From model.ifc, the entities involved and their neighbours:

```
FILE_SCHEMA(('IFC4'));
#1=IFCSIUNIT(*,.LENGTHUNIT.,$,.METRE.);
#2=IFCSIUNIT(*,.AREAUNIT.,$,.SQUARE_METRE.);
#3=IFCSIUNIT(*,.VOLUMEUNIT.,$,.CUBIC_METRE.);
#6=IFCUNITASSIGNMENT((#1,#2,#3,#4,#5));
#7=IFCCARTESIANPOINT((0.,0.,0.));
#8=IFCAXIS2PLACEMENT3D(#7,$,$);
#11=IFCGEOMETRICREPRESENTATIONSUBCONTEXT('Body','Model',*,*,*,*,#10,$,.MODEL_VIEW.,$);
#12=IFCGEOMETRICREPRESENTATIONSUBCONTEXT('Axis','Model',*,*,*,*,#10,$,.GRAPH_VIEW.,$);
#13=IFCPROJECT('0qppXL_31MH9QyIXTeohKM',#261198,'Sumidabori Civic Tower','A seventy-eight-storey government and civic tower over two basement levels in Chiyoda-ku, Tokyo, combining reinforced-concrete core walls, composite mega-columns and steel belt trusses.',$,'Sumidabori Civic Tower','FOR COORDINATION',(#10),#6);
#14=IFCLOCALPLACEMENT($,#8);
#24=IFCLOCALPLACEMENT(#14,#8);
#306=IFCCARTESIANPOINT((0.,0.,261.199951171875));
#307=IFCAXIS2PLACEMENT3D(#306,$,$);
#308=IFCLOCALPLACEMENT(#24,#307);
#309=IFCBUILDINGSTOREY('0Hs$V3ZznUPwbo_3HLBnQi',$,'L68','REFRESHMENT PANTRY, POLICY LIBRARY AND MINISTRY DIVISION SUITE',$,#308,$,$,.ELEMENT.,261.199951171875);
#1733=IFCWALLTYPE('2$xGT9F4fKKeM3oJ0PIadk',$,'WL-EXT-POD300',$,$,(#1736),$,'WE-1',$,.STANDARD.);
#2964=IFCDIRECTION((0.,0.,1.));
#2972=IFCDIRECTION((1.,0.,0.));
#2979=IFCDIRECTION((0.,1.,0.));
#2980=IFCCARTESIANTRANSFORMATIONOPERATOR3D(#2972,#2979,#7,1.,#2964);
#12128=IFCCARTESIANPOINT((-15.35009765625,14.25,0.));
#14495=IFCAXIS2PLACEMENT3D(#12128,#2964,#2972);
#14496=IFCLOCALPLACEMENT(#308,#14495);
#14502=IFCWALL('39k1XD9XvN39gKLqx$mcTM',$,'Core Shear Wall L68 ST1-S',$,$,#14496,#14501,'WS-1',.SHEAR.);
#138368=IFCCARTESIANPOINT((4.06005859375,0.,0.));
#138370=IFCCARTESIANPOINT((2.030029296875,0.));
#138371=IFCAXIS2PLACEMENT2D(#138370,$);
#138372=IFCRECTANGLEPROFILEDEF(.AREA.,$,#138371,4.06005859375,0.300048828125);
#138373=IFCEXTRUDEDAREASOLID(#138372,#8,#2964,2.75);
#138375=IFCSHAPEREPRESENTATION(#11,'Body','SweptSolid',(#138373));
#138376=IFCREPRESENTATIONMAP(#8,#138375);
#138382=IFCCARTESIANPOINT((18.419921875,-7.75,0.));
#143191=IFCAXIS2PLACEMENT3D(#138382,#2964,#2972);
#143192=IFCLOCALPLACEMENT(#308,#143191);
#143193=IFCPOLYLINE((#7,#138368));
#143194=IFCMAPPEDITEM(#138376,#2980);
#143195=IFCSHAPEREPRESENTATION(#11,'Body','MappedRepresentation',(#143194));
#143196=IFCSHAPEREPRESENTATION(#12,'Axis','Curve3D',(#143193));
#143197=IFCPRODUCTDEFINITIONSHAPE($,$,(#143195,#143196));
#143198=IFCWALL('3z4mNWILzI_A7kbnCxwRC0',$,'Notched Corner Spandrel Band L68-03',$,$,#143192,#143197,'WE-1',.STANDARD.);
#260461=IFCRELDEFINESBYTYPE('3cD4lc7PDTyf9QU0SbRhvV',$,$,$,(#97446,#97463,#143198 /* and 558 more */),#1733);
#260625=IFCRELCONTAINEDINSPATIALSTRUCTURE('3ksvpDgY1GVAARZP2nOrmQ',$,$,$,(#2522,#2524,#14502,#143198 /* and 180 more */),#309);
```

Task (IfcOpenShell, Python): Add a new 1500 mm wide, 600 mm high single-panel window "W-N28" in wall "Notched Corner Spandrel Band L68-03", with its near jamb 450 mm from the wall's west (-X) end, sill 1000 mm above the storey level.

```python
import numpy as np
import ifcopenshell
import ifcopenshell.api.feature
import ifcopenshell.api.geometry
import ifcopenshell.api.root
import ifcopenshell.api.spatial
import ifcopenshell.geom
import ifcopenshell.util.element
import ifcopenshell.util.placement
import ifcopenshell.util.representation
import ifcopenshell.util.shape
import ifcopenshell.util.unit

model = ifcopenshell.open("model.ifc")
unit_scale = ifcopenshell.util.unit.calculate_unit_scale(model)
settings = ifcopenshell.geom.settings()


def volume(element):
    """Net volume in cubic metres, openings subtracted."""
    shape = ifcopenshell.geom.create_shape(settings, element)
    return ifcopenshell.util.shape.get_volume(shape.geometry)


wall = model.by_guid("3z4mNWILzI_A7kbnCxwRC0")
storey = ifcopenshell.util.element.get_container(wall, ifc_class="IfcBuildingStorey")
context = ifcopenshell.util.representation.get_context(model, "Model", "Body", "MODEL_VIEW")
before = volume(wall)

width, height, from_end, sill = 1.5, 0.6, 0.45, 1  # metres

# The wall runs along its own X axis, and the end named is its -X end.
wall_shape = ifcopenshell.geom.create_shape(settings, wall)
x, y, z = ifcopenshell.util.shape.get_vertices(wall_shape.geometry).T
start = x.min() + from_end
face, thickness = float(y.min()), float(y.max() - y.min())
wall_matrix = ifcopenshell.util.placement.get_local_placement(wall.ObjectPlacement)
level = ifcopenshell.util.placement.get_local_placement(storey.ObjectPlacement)[2, 3]


def in_wall(x, y):
    """Placement at x, y metres in the wall's axes, at sill height."""
    matrix = wall_matrix.copy()
    matrix[:, 3] = wall_matrix @ np.array([x / unit_scale, y / unit_scale, 0.0, 1.0])
    matrix[2, 3] = level + sill / unit_scale
    return matrix


# Opening: a box that overshoots both wall faces by 50 mm.
opening = ifcopenshell.api.root.create_entity(model, ifc_class="IfcOpeningElement", predefined_type="OPENING")
box = ifcopenshell.api.geometry.add_wall_representation(
    model, context=context, length=width, height=height, thickness=thickness + 0.1
)
ifcopenshell.api.geometry.assign_representation(model, product=opening, representation=box)
ifcopenshell.api.geometry.edit_object_placement(model, product=opening, matrix=in_wall(start, face - 0.05), is_si=False)
ifcopenshell.api.feature.add_feature(model, feature=opening, element=wall)

window = ifcopenshell.api.root.create_entity(model, ifc_class="IfcWindow", name="W-N28", predefined_type="WINDOW")
window.OverallWidth, window.OverallHeight = width / unit_scale, height / unit_scale
window.PartitioningType = "SINGLE_PANEL"
body = ifcopenshell.api.geometry.add_window_representation(
    model,
    context=context,
    overall_width=window.OverallWidth,
    overall_height=window.OverallHeight,
    partition_type="SINGLE_PANEL",
)
ifcopenshell.api.geometry.assign_representation(model, product=window, representation=body)
ifcopenshell.api.spatial.assign_container(model, products=[window], relating_structure=storey)
ifcopenshell.api.feature.add_filling(model, opening=opening, element=window)

# Centre the window in the wall's thickness.
ifcopenshell.api.geometry.edit_object_placement(model, product=window, matrix=in_wall(start, face), is_si=False)
window_shape = ifcopenshell.geom.create_shape(settings, window)
depth = ifcopenshell.util.shape.get_vertices(window_shape.geometry)[:, 1]
offset = face + thickness / 2 - (depth.min() + depth.max()) / 2
ifcopenshell.api.geometry.edit_object_placement(model, product=window, matrix=in_wall(start, offset), is_si=False)

after = volume(wall)

print(f"wall volume {before:.3f} -> {after:.3f} m3")

model.write("model_edited.ifc")
```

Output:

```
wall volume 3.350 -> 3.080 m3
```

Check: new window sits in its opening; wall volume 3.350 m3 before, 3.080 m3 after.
